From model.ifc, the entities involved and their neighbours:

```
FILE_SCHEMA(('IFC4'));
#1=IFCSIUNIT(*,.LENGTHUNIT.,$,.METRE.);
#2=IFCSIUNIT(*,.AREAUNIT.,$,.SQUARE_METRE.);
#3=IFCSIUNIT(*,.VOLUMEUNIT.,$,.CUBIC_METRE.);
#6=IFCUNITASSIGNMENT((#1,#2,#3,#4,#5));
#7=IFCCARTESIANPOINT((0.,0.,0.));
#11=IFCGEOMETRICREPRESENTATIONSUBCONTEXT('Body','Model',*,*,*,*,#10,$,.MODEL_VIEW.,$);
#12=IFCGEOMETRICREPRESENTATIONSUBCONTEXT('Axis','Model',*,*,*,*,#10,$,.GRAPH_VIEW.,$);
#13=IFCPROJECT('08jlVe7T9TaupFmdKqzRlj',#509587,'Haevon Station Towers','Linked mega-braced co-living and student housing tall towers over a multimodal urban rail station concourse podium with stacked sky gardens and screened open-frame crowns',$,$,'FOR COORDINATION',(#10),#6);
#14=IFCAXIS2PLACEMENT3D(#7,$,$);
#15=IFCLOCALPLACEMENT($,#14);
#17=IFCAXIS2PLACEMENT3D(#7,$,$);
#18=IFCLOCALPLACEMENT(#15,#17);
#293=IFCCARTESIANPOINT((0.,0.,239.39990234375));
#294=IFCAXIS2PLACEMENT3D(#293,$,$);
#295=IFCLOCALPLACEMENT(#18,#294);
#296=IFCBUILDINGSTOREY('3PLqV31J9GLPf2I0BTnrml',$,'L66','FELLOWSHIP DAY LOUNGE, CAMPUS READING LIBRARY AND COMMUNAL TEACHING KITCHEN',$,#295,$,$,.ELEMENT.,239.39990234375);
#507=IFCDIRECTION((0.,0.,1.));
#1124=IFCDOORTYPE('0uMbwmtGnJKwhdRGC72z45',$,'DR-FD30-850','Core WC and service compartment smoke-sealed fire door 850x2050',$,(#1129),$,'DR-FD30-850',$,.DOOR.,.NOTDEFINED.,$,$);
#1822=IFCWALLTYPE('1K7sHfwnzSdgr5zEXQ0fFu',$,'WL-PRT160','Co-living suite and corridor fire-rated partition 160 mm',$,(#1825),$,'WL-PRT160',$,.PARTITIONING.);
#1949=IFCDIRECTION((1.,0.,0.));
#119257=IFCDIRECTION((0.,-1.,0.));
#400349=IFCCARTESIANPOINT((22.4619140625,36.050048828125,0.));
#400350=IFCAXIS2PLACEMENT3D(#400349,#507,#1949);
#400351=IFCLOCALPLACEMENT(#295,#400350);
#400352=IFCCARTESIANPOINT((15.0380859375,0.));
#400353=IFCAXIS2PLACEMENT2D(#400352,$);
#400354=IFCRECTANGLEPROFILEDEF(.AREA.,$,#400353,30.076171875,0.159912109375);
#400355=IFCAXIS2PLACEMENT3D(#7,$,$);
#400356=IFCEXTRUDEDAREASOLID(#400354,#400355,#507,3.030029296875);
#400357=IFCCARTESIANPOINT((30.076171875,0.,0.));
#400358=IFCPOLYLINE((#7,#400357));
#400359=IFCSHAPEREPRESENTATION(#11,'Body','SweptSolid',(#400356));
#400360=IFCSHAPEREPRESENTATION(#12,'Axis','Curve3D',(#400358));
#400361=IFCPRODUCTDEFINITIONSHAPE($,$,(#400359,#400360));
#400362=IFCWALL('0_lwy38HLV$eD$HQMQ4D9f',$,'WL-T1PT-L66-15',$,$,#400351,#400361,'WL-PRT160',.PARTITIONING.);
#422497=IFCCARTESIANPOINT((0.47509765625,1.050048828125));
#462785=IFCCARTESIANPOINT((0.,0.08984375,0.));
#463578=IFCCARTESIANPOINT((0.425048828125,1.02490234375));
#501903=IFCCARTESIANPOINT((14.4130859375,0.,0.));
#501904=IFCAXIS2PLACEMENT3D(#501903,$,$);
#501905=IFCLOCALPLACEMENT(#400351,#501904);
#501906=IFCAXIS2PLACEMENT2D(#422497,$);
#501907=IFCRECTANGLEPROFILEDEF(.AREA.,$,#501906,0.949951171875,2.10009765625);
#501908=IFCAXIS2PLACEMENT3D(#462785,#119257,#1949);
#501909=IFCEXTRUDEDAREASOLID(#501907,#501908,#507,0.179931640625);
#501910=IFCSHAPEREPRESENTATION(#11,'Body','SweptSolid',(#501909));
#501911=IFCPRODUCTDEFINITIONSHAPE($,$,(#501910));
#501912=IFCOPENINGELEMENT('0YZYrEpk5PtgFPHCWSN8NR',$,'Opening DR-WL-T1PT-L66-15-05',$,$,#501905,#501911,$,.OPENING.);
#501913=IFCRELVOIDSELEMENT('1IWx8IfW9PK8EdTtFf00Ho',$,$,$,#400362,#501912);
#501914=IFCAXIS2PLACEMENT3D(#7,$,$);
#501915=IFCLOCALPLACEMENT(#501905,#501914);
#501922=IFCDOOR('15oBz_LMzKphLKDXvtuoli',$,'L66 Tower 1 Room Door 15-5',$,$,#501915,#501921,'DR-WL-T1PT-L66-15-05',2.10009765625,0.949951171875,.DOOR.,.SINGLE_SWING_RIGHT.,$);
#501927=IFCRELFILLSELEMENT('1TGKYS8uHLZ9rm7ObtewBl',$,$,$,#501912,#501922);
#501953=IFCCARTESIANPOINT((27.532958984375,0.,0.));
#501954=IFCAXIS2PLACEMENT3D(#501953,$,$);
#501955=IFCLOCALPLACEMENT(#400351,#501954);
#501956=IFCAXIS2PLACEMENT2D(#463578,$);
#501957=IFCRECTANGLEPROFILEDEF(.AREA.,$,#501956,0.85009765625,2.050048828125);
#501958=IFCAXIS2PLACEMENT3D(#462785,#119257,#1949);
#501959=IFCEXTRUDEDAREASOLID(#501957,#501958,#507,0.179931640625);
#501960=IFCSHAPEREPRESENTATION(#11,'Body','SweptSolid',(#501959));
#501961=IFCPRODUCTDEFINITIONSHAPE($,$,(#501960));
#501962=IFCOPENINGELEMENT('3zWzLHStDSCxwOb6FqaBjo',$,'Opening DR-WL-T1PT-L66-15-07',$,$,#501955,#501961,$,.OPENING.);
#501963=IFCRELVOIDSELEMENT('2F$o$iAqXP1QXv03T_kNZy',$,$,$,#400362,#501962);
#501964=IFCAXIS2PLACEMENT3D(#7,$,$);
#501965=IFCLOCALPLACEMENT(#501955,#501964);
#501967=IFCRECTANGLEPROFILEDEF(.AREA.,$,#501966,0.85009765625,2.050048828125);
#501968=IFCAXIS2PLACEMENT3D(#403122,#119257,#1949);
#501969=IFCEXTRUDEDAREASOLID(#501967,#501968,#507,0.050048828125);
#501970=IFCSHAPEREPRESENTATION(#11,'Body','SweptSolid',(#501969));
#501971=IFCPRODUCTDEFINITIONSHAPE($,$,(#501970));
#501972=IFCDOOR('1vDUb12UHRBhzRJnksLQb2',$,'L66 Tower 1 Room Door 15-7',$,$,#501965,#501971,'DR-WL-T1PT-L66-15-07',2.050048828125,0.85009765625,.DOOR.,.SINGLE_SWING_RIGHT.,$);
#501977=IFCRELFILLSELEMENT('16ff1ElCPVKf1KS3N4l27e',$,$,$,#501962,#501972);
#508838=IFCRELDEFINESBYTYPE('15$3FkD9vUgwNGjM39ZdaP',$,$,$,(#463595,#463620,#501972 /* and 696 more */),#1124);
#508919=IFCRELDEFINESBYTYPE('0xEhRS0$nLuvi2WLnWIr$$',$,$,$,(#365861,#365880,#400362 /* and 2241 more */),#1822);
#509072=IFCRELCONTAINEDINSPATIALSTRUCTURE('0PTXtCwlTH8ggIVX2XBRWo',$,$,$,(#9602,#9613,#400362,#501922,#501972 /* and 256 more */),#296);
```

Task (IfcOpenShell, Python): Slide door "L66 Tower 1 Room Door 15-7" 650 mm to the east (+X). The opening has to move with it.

```python
import ifcopenshell
import ifcopenshell.api.geometry
import ifcopenshell.util.placement

model = ifcopenshell.open("model.ifc")

door = model.by_id(501972)
opening = door.FillsVoids[0].RelatingOpeningElement
wall = opening.VoidsElements[0].RelatingBuildingElement

wall_matrix = ifcopenshell.util.placement.get_local_placement(wall.ObjectPlacement)
shift = wall_matrix[:3, 0] * 0.65
before = ifcopenshell.util.placement.get_local_placement(door.ObjectPlacement)[:3, 3].copy()

# The door is placed relative to its opening, so it follows when the opening moves.
matrix = ifcopenshell.util.placement.get_local_placement(opening.ObjectPlacement)
matrix[:3, 3] += shift
ifcopenshell.api.geometry.edit_object_placement(
    model, product=opening, matrix=matrix, is_si=False, should_transform_children=True
)

after = ifcopenshell.util.placement.get_local_placement(door.ObjectPlacement)[:3, 3]
print("door moved by", (after - before).round(3) + 0.0)

model.write("model_rev.ifc")
```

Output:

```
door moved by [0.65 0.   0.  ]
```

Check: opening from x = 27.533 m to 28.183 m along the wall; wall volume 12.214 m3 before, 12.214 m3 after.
